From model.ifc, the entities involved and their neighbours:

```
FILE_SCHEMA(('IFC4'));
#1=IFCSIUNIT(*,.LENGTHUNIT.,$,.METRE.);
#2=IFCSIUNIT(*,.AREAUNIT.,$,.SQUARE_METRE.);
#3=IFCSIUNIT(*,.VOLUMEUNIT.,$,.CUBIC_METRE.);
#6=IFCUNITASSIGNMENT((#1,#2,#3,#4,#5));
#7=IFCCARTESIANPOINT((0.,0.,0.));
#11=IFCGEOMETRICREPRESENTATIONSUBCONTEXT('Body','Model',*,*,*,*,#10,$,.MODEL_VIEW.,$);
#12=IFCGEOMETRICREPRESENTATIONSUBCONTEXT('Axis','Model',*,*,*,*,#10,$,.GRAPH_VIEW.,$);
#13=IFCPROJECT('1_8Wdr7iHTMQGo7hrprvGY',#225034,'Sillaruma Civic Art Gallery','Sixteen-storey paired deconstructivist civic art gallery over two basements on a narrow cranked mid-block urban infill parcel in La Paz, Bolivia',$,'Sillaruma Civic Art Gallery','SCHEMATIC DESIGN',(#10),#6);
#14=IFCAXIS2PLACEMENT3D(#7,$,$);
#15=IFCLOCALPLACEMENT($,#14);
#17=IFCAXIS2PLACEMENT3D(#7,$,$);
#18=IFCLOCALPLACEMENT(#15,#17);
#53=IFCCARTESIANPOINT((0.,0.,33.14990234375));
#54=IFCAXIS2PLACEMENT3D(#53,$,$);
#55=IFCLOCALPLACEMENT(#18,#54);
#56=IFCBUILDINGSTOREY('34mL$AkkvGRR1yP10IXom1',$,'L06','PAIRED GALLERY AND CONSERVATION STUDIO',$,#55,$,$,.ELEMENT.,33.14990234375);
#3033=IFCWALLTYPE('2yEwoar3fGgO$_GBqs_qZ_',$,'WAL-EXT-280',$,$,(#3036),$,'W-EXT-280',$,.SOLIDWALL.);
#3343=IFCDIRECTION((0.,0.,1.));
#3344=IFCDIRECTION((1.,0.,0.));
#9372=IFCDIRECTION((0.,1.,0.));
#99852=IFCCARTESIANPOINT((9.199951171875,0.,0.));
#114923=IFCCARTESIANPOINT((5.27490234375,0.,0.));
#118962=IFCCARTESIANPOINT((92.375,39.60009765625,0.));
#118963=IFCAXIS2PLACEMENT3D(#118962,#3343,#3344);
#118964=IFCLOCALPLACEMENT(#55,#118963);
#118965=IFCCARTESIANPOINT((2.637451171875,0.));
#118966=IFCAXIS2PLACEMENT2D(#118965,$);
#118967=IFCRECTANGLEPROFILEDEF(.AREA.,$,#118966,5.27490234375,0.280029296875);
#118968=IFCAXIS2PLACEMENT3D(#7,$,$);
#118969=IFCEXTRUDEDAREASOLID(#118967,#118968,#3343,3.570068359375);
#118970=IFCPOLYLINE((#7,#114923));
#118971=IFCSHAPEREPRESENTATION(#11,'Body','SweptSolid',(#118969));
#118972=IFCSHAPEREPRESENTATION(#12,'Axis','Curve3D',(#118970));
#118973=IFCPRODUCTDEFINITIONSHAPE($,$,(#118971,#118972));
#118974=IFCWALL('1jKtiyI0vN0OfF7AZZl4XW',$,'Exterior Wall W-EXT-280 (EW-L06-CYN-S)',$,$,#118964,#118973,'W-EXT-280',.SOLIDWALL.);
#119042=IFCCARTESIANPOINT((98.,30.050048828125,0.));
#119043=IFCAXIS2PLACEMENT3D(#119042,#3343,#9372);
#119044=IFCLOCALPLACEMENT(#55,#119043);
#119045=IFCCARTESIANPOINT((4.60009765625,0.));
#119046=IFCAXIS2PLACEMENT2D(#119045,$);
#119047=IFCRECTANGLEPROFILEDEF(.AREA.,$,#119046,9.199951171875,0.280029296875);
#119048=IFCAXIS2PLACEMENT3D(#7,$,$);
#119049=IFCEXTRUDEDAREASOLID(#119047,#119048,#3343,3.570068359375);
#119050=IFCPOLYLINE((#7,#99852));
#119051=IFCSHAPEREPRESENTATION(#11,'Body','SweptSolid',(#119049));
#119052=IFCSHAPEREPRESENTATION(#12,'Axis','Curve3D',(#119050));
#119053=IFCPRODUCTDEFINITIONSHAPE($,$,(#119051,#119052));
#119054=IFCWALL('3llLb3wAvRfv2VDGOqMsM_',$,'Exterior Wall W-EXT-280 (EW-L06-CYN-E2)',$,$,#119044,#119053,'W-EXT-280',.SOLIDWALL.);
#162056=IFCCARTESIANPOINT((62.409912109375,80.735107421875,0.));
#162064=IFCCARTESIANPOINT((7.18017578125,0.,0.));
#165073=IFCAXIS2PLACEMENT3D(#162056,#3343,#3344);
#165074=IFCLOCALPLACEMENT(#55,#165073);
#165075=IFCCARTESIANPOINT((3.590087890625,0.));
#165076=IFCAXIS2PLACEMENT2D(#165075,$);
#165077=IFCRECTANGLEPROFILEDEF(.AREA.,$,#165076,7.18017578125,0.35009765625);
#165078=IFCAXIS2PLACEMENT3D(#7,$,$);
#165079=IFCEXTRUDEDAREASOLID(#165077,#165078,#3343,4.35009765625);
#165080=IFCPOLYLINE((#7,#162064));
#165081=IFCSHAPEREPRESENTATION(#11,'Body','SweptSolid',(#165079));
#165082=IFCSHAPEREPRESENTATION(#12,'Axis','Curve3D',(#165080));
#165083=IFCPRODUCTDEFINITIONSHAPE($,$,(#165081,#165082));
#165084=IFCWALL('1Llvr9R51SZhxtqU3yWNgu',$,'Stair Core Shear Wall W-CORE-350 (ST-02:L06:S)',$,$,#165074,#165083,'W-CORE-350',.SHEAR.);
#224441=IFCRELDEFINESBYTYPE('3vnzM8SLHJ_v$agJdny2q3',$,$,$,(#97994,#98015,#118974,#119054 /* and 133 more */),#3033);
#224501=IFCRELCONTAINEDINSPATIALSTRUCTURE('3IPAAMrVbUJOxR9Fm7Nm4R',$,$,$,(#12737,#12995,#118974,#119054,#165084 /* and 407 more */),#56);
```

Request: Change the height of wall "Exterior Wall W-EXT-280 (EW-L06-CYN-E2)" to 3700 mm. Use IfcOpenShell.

```python
import ifcopenshell
import ifcopenshell.geom
import ifcopenshell.util.representation
import ifcopenshell.util.shape

model = ifcopenshell.open("model.ifc")
settings = ifcopenshell.geom.settings()


def volume(element):
    """Net volume in cubic metres, openings subtracted."""
    shape = ifcopenshell.geom.create_shape(settings, element)
    return ifcopenshell.util.shape.get_volume(shape.geometry)


wall = model.by_id(119054)
before = volume(wall)

body = ifcopenshell.util.representation.get_representation(wall, "Model", "Body")
solid = body.Items[0]
old_height = solid.Depth
solid.Depth = 3.7
after = volume(wall)

print(f"height {old_height:g} -> {solid.Depth:g}, volume {before:.3f} -> {after:.3f} m3")

model.write("model_v2.ifc")
```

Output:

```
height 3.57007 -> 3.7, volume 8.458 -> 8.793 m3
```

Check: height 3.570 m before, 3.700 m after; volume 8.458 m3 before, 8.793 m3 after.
